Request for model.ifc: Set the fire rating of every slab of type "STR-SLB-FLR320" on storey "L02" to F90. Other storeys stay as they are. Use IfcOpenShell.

First a look at what the model holds.

```python
import ifcopenshell
import ifcopenshell.util.element

model = ifcopenshell.open("model.ifc")
print(model.schema)
storey = next(s for s in model.by_type("IfcBuildingStorey") if s.Name == "L02")
slabs = [e for e in ifcopenshell.util.element.get_decomposition(storey) if e.is_a("IfcSlab")]
seen = {}
for e in slabs:
    element_type = ifcopenshell.util.element.get_type(e)
    key = (element_type.Name if element_type != e and element_type else None, ifcopenshell.util.element.get_pset(e, "Pset_SlabCommon", "FireRating"))
    seen[key] = seen.get(key, 0) + 1
for (name, value), count in sorted(seen.items(), key=str):
    print(count, "x", name, "|", value)
```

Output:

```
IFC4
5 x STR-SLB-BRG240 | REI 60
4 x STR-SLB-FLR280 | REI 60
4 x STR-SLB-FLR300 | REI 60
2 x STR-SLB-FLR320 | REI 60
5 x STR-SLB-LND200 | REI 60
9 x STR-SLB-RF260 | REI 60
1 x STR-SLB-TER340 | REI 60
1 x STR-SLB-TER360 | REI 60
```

```python
import ifcopenshell
import ifcopenshell.api.pset
import ifcopenshell.util.element

model = ifcopenshell.open("model.ifc")

storey = next(s for s in model.by_type("IfcBuildingStorey") if s.Name == "L02")
slabs = [e for e in ifcopenshell.util.element.get_decomposition(storey) if e.is_a("IfcSlab")]

count = 0
for e in slabs:
    element_type = ifcopenshell.util.element.get_type(e)
    if element_type in (None, e) or element_type.Name != "STR-SLB-FLR320":
        continue
    # add_pset returns the element's existing set when there is one.
    pset = ifcopenshell.api.pset.add_pset(model, product=e, name="Pset_SlabCommon")
    ifcopenshell.api.pset.edit_pset(model, pset=pset, properties={"FireRating": "F90"})
    count += 1

print(count, "slabs updated")

model.write("model_v2.ifc")
```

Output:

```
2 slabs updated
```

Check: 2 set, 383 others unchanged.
